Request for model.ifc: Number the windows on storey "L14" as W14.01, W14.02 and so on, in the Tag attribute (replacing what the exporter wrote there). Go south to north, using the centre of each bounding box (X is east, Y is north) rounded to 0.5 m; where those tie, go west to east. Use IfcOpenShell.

First a look at what the model holds.

```python
import ifcopenshell
import ifcopenshell.util.element
import ifcopenshell.util.placement

model = ifcopenshell.open("model.ifc")
print(model.schema)
storey = next(s for s in model.by_type("IfcBuildingStorey") if s.Name == "L14")
windows = [e for e in ifcopenshell.util.element.get_decomposition(storey) if e.is_a("IfcWindow")]
for e in sorted(windows, key=lambda e: e.id()):
    origin = ifcopenshell.util.placement.get_local_placement(e.ObjectPlacement)[:3, 3]
    print(e.id(), e.Tag, e.Name, origin.round(2) + 0.0, sep=" | ")
```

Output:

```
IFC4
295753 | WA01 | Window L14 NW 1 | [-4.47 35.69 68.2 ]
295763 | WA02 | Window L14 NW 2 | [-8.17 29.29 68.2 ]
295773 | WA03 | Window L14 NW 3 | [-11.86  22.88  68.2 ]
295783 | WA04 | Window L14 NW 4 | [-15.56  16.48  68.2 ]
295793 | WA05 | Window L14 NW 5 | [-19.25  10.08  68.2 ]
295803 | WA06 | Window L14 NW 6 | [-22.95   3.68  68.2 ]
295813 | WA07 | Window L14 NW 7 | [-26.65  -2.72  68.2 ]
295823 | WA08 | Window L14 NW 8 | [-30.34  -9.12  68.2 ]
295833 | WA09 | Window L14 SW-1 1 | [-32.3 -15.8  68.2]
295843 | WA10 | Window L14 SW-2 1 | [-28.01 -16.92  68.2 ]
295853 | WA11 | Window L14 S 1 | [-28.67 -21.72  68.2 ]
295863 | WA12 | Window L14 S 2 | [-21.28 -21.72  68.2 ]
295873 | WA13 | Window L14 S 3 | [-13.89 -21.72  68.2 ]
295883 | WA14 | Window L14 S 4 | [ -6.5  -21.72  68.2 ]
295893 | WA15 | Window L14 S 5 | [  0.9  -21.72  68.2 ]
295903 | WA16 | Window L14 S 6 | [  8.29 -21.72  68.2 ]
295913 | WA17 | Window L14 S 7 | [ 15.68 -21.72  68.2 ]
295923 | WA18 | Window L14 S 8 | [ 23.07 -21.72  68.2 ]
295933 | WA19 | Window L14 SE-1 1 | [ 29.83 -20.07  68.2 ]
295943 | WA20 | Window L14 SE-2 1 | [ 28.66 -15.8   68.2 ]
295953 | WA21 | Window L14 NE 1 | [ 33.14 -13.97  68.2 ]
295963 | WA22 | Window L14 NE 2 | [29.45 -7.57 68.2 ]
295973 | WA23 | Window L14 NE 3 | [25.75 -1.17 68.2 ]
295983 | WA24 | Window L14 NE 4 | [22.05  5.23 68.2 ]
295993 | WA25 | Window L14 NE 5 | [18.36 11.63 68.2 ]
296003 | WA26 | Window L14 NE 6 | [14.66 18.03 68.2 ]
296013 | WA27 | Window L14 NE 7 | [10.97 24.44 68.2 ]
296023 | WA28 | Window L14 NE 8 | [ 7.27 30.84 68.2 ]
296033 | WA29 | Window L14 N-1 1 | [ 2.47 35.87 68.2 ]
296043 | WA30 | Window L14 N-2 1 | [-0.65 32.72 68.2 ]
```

```python
import ifcopenshell
import ifcopenshell.geom
import ifcopenshell.util.element
import ifcopenshell.util.shape

model = ifcopenshell.open("model.ifc")
settings = ifcopenshell.geom.settings()
settings.set("use-world-coords", True)


def centre(element):
    shape = ifcopenshell.geom.create_shape(settings, element)
    return ifcopenshell.util.shape.get_bbox_centroid(shape.geometry)


storey = next(s for s in model.by_type("IfcBuildingStorey") if s.Name == "L14")
windows = [e for e in ifcopenshell.util.element.get_decomposition(storey) if e.is_a("IfcWindow")]

# Insertion points can sit at a corner or the storey origin, so sort by the geometry (in metres).
centres = {e: centre(e) for e in windows}
windows.sort(key=lambda e: (round(centres[e][1] / 0.5), centres[e][0]))

for i, e in enumerate(windows, start=1):
    number = f"W14.{i:02d}"
    e.Tag = number
    print(e.id(), number)

model.write("model_v2.ifc")
```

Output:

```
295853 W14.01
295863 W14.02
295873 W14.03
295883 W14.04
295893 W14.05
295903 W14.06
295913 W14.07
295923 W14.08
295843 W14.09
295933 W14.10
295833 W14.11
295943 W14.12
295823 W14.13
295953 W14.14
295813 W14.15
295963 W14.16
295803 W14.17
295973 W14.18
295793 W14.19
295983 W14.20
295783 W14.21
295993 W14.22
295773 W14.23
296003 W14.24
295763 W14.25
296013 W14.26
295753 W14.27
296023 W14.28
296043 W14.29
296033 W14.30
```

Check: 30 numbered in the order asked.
